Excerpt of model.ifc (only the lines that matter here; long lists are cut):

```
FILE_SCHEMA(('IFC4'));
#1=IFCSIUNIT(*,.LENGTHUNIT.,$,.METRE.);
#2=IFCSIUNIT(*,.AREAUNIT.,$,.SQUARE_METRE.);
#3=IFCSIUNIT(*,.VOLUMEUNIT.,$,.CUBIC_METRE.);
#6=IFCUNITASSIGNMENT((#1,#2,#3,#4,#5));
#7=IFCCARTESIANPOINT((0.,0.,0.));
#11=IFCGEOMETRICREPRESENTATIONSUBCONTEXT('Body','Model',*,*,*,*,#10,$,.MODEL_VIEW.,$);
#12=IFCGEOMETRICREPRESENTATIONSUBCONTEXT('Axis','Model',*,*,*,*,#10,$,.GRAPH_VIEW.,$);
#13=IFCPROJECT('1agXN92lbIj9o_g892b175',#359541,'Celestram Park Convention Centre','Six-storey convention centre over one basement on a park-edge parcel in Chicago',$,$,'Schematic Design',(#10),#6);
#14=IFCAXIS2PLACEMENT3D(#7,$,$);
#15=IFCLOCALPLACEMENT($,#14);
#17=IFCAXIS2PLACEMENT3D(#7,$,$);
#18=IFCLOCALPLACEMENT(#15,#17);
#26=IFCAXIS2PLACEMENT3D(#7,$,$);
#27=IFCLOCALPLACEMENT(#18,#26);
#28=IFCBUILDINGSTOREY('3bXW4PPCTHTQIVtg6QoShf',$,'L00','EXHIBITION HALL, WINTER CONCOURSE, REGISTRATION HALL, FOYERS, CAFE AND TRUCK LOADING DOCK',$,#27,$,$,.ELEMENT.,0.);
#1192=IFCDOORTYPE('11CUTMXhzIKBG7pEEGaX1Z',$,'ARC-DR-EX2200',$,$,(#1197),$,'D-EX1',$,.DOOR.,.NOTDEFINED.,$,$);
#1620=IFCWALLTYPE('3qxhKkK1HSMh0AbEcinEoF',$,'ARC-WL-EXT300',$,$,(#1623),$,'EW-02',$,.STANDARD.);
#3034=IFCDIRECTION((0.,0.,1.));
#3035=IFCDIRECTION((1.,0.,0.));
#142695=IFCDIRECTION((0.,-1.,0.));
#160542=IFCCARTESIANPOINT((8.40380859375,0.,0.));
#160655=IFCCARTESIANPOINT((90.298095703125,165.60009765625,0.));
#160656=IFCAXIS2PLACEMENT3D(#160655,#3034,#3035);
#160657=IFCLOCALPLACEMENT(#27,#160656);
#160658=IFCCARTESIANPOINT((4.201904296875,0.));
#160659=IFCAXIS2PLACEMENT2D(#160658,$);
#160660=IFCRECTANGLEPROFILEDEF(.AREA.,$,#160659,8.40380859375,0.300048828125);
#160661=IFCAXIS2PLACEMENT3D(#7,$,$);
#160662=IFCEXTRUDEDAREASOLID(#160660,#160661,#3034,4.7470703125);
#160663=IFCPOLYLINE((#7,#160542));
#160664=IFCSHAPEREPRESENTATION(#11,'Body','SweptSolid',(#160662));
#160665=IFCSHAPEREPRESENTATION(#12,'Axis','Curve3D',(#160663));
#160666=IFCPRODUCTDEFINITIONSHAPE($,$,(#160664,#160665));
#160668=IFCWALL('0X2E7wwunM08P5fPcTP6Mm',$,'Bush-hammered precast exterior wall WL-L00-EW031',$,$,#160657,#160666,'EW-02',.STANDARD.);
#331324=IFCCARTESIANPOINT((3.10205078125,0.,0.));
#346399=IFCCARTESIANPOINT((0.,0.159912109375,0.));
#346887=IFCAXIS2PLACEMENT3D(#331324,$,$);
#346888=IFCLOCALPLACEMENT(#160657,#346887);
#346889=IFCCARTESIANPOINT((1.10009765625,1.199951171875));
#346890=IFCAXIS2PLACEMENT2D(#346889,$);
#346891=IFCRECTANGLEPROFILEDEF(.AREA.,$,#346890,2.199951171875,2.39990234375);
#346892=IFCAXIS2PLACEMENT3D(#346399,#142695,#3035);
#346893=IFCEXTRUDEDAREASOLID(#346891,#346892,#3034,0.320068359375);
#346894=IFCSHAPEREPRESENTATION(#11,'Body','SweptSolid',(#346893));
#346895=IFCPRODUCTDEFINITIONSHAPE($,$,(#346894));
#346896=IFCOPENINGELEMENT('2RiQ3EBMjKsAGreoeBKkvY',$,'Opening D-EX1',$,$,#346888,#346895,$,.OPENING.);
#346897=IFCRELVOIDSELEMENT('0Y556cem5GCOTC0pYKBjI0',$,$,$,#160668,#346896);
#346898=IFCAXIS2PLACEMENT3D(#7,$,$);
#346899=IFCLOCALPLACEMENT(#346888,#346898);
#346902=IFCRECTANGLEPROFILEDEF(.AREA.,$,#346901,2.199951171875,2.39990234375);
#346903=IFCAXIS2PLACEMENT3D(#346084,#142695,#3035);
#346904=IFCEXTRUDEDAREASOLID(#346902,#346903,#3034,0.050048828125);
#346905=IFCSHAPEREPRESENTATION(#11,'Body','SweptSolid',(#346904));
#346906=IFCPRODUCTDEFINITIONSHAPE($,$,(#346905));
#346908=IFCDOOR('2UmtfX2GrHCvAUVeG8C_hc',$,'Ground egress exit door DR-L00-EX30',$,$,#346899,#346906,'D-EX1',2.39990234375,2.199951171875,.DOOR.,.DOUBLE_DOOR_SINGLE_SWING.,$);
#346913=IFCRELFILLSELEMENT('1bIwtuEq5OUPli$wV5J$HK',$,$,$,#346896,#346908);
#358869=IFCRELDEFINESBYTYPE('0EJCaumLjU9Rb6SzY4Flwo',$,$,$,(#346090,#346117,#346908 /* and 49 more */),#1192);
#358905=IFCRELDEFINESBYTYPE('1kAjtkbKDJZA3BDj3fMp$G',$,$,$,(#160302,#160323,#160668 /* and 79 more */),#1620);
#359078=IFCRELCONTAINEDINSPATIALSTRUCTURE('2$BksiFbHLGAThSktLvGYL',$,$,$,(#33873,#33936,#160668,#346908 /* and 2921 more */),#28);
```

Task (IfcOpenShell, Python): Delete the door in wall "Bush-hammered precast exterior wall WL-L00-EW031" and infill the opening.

```python
import ifcopenshell
import ifcopenshell.api.feature
import ifcopenshell.api.root
import ifcopenshell.geom
import ifcopenshell.util.shape

model = ifcopenshell.open("model.ifc")
settings = ifcopenshell.geom.settings()


def volume(element):
    """Net volume in cubic metres, openings subtracted."""
    shape = ifcopenshell.geom.create_shape(settings, element)
    return ifcopenshell.util.shape.get_volume(shape.geometry)


door = model.by_guid("2UmtfX2GrHCvAUVeG8C_hc")
opening = door.FillsVoids[0].RelatingOpeningElement
wall = opening.VoidsElements[0].RelatingBuildingElement
before = volume(wall)

ifcopenshell.api.root.remove_product(model, product=door)
ifcopenshell.api.feature.remove_feature(model, feature=opening)

after = volume(wall)

print(f"wall volume {before:.3f} -> {after:.3f} m3")

model.write("model_edited.ifc")
```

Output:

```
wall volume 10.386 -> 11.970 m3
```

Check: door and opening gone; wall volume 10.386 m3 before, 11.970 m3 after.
